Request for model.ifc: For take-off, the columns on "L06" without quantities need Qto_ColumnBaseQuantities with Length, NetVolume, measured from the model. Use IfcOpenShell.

First a look at what the model holds.

```python
import ifcopenshell
import ifcopenshell.util.element
import ifcopenshell.util.unit

model = ifcopenshell.open("model.ifc")
print(model.schema)
for unit_type in ("LENGTHUNIT", "AREAUNIT", "VOLUMEUNIT"):
    print(unit_type, ifcopenshell.util.unit.calculate_unit_scale(model, unit_type))
storey = next(s for s in model.by_type("IfcBuildingStorey") if s.Name == "L06")
columns = [e for e in ifcopenshell.util.element.get_decomposition(storey) if e.is_a("IfcColumn")]
for e in sorted(columns, key=lambda e: e.id()):
    print(e.id(), e.is_a(), e.Name, list(ifcopenshell.util.element.get_psets(e, qtos_only=True)), sep=" | ")
```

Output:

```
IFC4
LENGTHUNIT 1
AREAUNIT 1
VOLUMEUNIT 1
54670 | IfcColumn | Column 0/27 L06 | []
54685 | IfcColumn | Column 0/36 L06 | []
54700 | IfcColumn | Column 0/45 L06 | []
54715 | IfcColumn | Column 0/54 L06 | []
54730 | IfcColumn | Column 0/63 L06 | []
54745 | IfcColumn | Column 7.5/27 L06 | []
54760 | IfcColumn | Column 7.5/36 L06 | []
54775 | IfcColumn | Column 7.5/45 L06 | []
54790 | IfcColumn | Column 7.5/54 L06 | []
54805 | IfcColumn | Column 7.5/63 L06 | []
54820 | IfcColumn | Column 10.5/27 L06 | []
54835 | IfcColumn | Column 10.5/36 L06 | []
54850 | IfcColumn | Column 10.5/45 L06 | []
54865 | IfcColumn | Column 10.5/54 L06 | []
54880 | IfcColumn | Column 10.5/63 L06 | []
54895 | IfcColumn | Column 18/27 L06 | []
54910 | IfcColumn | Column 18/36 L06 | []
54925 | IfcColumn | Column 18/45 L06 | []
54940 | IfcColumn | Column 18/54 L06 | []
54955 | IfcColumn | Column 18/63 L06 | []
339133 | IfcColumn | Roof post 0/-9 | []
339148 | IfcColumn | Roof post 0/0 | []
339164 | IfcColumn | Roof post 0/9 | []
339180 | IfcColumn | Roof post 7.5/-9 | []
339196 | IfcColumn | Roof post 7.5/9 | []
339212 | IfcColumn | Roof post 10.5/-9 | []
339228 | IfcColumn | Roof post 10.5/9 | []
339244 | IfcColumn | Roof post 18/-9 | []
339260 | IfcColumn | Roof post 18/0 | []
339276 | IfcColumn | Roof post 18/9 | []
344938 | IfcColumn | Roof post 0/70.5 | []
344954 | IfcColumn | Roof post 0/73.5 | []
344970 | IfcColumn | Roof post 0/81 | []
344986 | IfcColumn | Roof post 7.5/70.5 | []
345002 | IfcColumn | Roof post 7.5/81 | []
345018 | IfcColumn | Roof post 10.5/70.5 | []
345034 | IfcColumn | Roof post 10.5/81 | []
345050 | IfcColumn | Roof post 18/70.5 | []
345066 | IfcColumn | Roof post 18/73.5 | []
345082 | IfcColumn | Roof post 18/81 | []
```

```python
import ifcopenshell
import ifcopenshell.api.pset
import ifcopenshell.geom
import ifcopenshell.util.element
import ifcopenshell.util.shape
import ifcopenshell.util.unit

model = ifcopenshell.open("model.ifc")
unit_scale = ifcopenshell.util.unit.calculate_unit_scale(model)
volume_scale = ifcopenshell.util.unit.calculate_unit_scale(model, "VOLUMEUNIT")
settings = ifcopenshell.geom.settings()

storey = next(s for s in model.by_type("IfcBuildingStorey") if s.Name == "L06")
columns = [e for e in ifcopenshell.util.element.get_decomposition(storey) if e.is_a("IfcColumn")]

for e in sorted(columns, key=lambda e: e.id()):
    if ifcopenshell.util.element.get_psets(e, qtos_only=True, should_inherit=False):
        continue
    # Geometry comes back in metres, in the element's own axes.
    shape = ifcopenshell.geom.create_shape(settings, e)
    values = {
        "Length": ifcopenshell.util.shape.get_z(shape.geometry) / unit_scale,
        "NetVolume": ifcopenshell.util.shape.get_volume(shape.geometry) / volume_scale,
    }
    qto = ifcopenshell.api.pset.add_qto(model, product=e, name="Qto_ColumnBaseQuantities")
    ifcopenshell.api.pset.edit_qto(model, qto=qto, properties=values)
    print(e.id(), {k: round(v, 3) for k, v in values.items()})

model.write("model_updated.ifc")
```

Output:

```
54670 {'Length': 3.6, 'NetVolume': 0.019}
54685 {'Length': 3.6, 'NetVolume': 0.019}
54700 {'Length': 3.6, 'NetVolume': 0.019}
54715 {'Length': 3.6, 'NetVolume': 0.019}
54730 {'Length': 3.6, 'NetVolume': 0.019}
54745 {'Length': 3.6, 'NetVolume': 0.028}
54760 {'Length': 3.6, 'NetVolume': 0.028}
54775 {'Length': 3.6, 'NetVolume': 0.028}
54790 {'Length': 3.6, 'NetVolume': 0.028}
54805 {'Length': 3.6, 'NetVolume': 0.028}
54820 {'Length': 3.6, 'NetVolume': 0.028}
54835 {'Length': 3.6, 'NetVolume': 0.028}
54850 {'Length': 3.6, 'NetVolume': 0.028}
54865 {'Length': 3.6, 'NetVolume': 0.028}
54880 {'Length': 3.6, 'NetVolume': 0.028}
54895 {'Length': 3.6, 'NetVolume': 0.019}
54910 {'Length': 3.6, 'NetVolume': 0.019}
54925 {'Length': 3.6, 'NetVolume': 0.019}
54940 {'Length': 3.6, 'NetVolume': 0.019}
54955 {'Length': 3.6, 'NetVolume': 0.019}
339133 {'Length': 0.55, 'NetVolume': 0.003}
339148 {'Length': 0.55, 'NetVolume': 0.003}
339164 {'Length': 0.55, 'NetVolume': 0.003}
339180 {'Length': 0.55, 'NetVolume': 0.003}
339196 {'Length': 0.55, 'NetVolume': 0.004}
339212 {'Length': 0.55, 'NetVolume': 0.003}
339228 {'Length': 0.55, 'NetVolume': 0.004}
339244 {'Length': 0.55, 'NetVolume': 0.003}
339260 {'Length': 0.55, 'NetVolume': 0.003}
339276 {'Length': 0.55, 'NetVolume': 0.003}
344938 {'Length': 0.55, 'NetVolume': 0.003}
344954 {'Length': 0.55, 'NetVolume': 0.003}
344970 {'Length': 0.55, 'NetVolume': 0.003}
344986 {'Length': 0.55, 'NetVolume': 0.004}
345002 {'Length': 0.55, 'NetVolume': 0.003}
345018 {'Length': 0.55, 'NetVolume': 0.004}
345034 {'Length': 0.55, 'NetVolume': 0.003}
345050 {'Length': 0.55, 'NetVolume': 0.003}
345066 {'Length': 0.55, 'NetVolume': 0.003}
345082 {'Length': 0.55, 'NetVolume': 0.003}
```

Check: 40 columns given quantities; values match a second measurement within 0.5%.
